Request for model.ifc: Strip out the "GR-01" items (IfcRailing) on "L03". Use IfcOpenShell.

First a look at what the model holds.

```python
import ifcopenshell
import ifcopenshell.util.element

model = ifcopenshell.open("model.ifc")
print(model.schema)
storey = next(s for s in model.by_type("IfcBuildingStorey") if s.Name == "L03")
railings = [e for e in ifcopenshell.util.element.get_decomposition(storey) if e.is_a("IfcRailing")]
seen = {}
for e in railings:
    element_type = ifcopenshell.util.element.get_type(e)
    name = element_type.Name if element_type not in (None, e) else None
    seen[name] = seen.get(name, 0) + 1
for name, count in sorted(seen.items(), key=str):
    print(count, "x", name)
```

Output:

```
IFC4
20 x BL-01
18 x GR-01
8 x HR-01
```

```python
import ifcopenshell
import ifcopenshell.api.root
import ifcopenshell.util.element

model = ifcopenshell.open("model.ifc")

storey = next(s for s in model.by_type("IfcBuildingStorey") if s.Name == "L03")
railings = [e for e in ifcopenshell.util.element.get_decomposition(storey) if e.is_a("IfcRailing")]
targets = [e for e in railings if (t := ifcopenshell.util.element.get_type(e)) not in (None, e) and t.Name == "GR-01"]

for e in targets:
    ifcopenshell.api.root.remove_product(model, product=e)
print(len(targets), "removed")

model.write("model-out.ifc")
```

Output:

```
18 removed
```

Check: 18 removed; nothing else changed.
